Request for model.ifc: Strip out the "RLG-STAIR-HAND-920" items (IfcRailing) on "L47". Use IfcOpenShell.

First a look at what the model holds.

```python
import ifcopenshell
import ifcopenshell.util.element

model = ifcopenshell.open("model.ifc")
print(model.schema)
storey = next(s for s in model.by_type("IfcBuildingStorey") if s.Name == "L47")
railings = [e for e in ifcopenshell.util.element.get_decomposition(storey) if e.is_a("IfcRailing")]
seen = {}
for e in railings:
    element_type = ifcopenshell.util.element.get_type(e)
    name = element_type.Name if element_type not in (None, e) else None
    seen[name] = seen.get(name, 0) + 1
for name, count in sorted(seen.items(), key=str):
    print(count, "x", name)
```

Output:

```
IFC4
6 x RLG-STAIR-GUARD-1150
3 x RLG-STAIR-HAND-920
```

```python
import ifcopenshell
import ifcopenshell.api.root
import ifcopenshell.util.element

model = ifcopenshell.open("model.ifc")

storey = next(s for s in model.by_type("IfcBuildingStorey") if s.Name == "L47")
railings = [e for e in ifcopenshell.util.element.get_decomposition(storey) if e.is_a("IfcRailing")]
targets = [e for e in railings if (t := ifcopenshell.util.element.get_type(e)) not in (None, e) and t.Name == "RLG-STAIR-HAND-920"]

for e in targets:
    ifcopenshell.api.root.remove_product(model, product=e)
print(len(targets), "removed")

model.write("model-out.ifc")
```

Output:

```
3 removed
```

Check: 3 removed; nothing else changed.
